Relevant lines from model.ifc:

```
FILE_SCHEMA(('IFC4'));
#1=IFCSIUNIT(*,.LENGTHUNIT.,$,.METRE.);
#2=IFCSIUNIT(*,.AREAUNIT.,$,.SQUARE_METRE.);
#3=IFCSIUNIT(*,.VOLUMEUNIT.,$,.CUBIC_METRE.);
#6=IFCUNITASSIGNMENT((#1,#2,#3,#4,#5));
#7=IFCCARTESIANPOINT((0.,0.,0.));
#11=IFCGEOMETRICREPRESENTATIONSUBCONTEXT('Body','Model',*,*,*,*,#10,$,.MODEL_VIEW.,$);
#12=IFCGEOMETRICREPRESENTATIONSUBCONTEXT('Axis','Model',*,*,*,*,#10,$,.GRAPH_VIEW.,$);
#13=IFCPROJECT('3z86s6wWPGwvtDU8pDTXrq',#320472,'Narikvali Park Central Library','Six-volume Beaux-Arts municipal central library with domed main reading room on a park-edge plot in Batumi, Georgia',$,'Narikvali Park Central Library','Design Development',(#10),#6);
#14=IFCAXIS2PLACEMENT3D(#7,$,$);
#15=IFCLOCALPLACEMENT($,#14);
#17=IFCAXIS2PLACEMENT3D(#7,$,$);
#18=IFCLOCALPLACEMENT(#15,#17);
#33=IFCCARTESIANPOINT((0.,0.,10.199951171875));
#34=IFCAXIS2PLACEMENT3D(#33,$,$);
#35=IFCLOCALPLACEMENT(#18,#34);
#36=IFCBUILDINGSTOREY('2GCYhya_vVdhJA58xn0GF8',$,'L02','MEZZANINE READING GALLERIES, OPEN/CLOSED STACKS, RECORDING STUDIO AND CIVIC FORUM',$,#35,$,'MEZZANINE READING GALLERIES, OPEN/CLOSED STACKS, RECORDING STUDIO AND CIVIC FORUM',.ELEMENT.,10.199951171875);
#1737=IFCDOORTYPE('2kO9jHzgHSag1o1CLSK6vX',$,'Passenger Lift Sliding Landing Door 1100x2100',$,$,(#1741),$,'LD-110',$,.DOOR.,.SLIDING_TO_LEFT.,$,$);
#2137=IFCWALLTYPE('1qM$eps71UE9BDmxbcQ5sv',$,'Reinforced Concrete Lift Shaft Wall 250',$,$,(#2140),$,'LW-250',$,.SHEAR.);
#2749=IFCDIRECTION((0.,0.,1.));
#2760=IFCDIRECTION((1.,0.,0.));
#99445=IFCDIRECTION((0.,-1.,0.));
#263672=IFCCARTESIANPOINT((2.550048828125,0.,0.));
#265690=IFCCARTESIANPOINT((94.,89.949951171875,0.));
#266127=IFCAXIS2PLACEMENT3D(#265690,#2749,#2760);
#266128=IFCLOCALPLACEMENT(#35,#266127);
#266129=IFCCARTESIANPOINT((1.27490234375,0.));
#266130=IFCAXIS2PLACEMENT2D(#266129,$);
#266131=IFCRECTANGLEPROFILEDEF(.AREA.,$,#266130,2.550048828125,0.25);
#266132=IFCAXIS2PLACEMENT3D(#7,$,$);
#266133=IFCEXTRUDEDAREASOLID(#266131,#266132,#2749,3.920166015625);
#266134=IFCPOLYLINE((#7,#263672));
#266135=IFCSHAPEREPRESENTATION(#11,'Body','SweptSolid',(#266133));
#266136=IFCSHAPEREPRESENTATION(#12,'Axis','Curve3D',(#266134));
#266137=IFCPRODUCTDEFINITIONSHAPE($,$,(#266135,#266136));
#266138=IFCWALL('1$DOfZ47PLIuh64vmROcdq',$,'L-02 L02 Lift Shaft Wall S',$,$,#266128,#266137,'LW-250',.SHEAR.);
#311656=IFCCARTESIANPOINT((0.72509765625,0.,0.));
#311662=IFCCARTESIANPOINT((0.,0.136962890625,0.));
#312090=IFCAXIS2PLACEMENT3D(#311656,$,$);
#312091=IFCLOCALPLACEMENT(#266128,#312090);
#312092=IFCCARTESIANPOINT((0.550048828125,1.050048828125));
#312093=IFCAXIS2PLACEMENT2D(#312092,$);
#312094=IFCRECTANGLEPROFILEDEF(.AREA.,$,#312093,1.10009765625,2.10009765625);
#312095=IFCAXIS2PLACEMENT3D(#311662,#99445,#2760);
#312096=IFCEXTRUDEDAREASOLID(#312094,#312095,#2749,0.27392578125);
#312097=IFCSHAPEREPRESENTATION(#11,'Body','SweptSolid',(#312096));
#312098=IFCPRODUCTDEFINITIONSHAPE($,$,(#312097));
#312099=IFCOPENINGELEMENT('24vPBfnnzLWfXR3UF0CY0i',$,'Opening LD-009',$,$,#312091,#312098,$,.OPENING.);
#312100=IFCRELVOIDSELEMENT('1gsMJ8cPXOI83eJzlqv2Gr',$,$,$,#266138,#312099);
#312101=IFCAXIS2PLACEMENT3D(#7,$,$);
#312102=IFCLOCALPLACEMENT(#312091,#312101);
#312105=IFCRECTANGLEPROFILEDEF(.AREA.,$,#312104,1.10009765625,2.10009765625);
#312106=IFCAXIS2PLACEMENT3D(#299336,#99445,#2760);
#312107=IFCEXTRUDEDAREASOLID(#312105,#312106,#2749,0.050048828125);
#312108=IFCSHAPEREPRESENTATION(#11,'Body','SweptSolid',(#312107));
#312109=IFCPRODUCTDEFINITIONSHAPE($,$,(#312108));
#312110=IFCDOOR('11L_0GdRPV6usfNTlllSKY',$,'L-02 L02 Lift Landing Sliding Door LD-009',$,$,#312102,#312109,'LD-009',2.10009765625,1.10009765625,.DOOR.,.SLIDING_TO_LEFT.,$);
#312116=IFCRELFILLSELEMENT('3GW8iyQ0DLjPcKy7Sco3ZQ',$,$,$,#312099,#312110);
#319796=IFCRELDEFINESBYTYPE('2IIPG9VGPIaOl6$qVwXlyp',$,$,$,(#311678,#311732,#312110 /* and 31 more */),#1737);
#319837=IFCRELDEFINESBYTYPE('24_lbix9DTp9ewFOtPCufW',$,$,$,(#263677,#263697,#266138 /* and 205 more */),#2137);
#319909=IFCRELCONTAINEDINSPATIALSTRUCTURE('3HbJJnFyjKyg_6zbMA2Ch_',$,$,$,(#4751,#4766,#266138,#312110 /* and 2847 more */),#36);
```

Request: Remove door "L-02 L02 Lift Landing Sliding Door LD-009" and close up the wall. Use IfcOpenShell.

```python
import ifcopenshell
import ifcopenshell.api.feature
import ifcopenshell.api.root
import ifcopenshell.geom
import ifcopenshell.util.shape

model = ifcopenshell.open("model.ifc")
settings = ifcopenshell.geom.settings()


def volume(element):
    """Net volume in cubic metres, openings subtracted."""
    shape = ifcopenshell.geom.create_shape(settings, element)
    return ifcopenshell.util.shape.get_volume(shape.geometry)


door = model.by_guid("11L_0GdRPV6usfNTlllSKY")
opening = door.FillsVoids[0].RelatingOpeningElement
wall = opening.VoidsElements[0].RelatingBuildingElement
before = volume(wall)

ifcopenshell.api.root.remove_product(model, product=door)
ifcopenshell.api.feature.remove_feature(model, feature=opening)

after = volume(wall)

print(f"wall volume {before:.3f} -> {after:.3f} m3")

model.write("model_updated.ifc")
```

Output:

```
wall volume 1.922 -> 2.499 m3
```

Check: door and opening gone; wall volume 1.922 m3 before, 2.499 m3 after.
